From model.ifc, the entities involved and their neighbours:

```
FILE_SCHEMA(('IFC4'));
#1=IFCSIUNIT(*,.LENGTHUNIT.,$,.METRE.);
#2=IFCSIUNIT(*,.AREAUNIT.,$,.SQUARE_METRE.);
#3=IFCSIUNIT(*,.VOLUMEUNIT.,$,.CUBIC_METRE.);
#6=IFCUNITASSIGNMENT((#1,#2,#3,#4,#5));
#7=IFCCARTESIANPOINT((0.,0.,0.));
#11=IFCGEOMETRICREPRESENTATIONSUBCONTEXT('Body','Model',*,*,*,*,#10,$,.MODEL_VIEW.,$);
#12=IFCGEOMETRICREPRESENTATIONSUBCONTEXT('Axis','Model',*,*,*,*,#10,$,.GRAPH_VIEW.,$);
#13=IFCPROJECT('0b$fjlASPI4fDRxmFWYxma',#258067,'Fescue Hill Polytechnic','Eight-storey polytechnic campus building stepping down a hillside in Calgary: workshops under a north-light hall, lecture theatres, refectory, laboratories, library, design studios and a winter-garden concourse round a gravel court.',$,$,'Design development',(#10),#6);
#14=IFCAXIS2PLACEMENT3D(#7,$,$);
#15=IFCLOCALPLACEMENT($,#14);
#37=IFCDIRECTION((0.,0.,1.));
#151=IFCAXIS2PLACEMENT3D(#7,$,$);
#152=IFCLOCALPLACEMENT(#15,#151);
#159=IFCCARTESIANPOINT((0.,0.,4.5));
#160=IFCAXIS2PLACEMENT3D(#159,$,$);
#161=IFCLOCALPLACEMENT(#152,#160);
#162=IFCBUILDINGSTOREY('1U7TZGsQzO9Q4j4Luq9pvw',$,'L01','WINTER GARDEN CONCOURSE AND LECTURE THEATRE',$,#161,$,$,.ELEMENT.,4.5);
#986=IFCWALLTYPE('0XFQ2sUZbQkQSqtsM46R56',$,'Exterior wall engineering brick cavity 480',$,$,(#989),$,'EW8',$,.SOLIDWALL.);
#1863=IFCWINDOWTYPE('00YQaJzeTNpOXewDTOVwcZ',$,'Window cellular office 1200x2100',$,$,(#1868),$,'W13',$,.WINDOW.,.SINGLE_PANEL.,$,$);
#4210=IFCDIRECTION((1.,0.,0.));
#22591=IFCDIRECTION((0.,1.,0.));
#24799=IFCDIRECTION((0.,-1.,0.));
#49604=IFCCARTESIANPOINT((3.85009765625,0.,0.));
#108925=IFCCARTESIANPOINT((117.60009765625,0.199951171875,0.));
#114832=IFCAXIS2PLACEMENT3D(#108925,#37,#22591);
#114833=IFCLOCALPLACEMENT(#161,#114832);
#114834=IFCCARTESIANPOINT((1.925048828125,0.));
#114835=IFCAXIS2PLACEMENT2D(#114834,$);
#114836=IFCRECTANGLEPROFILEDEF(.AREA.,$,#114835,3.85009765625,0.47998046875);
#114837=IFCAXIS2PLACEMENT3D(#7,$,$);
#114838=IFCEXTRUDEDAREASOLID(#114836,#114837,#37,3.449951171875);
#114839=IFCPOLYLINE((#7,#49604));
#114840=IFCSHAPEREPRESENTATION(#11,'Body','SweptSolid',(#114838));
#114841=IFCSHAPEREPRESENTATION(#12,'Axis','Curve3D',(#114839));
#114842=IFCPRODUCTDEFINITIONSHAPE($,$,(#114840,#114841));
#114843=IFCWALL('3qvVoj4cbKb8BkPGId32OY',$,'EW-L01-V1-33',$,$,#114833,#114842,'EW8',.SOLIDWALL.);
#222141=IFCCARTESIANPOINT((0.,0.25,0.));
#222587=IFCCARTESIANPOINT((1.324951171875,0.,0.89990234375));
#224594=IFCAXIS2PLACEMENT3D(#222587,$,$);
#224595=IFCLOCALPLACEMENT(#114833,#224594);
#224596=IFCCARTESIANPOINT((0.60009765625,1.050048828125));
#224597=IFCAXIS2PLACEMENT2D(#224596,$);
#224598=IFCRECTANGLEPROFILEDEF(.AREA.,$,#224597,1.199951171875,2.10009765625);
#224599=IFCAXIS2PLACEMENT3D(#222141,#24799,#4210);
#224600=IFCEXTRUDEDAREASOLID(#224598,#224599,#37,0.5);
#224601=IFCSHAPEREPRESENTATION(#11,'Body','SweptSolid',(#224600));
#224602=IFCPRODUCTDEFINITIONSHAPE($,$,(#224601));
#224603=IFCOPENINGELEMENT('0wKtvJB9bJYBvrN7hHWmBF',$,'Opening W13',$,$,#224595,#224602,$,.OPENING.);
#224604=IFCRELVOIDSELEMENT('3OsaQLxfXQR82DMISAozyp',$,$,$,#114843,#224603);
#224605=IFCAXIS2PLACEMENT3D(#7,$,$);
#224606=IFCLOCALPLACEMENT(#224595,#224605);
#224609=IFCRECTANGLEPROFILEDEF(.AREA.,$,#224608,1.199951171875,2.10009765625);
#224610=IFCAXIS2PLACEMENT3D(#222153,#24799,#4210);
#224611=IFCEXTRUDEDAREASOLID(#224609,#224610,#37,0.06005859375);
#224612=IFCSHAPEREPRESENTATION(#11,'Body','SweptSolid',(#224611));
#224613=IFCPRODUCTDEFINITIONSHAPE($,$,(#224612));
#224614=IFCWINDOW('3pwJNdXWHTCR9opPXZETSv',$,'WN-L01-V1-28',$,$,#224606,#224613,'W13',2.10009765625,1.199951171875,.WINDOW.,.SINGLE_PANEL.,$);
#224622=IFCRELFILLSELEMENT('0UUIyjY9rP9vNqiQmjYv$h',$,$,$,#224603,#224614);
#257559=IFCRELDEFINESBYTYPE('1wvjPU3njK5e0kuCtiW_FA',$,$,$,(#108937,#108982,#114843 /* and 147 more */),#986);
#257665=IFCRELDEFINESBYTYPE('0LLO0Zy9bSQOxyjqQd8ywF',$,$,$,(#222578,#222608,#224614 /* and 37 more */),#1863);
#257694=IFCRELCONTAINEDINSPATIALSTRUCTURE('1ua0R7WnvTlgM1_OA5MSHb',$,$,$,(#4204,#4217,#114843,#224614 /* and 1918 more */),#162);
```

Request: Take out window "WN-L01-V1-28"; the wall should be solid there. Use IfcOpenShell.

```python
import ifcopenshell
import ifcopenshell.api.feature
import ifcopenshell.api.root
import ifcopenshell.geom
import ifcopenshell.util.shape

model = ifcopenshell.open("model.ifc")
settings = ifcopenshell.geom.settings()


def volume(element):
    """Net volume in cubic metres, openings subtracted."""
    shape = ifcopenshell.geom.create_shape(settings, element)
    return ifcopenshell.util.shape.get_volume(shape.geometry)


window = model.by_guid("3pwJNdXWHTCR9opPXZETSv")
opening = window.FillsVoids[0].RelatingOpeningElement
wall = opening.VoidsElements[0].RelatingBuildingElement
before = volume(wall)

ifcopenshell.api.root.remove_product(model, product=window)
ifcopenshell.api.feature.remove_feature(model, feature=opening)

after = volume(wall)

print(f"wall volume {before:.3f} -> {after:.3f} m3")

model.write("model_updated.ifc")
```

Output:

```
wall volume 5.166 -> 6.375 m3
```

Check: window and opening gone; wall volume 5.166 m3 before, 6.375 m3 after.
